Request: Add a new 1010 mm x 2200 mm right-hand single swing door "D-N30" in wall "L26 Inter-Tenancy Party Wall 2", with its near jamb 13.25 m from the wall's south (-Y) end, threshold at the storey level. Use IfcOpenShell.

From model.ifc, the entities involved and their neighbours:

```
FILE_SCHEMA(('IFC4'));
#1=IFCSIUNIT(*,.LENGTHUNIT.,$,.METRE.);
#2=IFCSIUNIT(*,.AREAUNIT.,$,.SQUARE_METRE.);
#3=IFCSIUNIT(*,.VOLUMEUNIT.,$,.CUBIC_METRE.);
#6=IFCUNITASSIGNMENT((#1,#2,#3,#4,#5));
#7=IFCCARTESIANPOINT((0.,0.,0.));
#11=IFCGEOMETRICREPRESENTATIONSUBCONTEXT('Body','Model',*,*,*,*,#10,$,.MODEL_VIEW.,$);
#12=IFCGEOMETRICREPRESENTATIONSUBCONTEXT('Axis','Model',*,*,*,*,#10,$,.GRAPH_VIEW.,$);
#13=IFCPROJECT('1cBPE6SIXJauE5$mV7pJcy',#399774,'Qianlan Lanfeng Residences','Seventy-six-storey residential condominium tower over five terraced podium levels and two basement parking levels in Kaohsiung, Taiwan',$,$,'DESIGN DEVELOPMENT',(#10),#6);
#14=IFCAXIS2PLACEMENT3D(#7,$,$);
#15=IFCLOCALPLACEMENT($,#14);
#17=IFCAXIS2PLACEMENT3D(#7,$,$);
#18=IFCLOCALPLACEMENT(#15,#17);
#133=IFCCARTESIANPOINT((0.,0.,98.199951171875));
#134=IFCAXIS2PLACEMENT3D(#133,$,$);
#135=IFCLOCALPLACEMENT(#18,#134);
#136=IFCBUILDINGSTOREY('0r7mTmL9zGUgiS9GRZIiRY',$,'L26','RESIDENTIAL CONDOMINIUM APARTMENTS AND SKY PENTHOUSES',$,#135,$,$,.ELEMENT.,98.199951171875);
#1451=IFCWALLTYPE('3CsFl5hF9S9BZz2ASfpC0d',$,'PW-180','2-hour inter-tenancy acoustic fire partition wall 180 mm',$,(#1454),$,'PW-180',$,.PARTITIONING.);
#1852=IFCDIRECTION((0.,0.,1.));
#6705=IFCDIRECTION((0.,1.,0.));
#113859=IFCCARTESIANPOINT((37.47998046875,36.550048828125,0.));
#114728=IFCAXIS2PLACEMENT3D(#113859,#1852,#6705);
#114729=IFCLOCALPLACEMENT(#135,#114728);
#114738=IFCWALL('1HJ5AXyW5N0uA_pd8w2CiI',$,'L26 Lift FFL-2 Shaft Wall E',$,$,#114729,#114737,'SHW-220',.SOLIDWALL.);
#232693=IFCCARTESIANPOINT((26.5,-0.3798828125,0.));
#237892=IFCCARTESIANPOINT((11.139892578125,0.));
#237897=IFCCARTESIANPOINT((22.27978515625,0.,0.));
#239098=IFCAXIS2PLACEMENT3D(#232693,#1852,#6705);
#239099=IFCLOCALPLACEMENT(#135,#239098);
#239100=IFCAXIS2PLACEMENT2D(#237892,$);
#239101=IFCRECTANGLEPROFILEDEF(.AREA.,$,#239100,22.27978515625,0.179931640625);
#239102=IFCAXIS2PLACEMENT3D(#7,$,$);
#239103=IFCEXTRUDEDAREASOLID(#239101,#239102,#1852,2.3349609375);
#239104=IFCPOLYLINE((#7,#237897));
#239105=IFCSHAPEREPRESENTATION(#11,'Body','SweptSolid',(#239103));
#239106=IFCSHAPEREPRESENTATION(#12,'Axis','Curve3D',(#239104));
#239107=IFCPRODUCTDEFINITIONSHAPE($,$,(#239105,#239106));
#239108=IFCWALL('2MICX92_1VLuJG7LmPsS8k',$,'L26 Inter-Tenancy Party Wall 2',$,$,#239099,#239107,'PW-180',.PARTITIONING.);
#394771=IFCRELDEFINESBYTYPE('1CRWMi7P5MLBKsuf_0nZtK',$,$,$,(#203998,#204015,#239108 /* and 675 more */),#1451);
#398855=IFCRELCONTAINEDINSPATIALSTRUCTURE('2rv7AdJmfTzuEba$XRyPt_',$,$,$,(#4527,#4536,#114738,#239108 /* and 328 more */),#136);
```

```python
import numpy as np
import ifcopenshell
import ifcopenshell.api.feature
import ifcopenshell.api.geometry
import ifcopenshell.api.root
import ifcopenshell.api.spatial
import ifcopenshell.geom
import ifcopenshell.util.element
import ifcopenshell.util.placement
import ifcopenshell.util.representation
import ifcopenshell.util.shape
import ifcopenshell.util.unit

model = ifcopenshell.open("model.ifc")
unit_scale = ifcopenshell.util.unit.calculate_unit_scale(model)
settings = ifcopenshell.geom.settings()


def volume(element):
    """Net volume in cubic metres, openings subtracted."""
    shape = ifcopenshell.geom.create_shape(settings, element)
    return ifcopenshell.util.shape.get_volume(shape.geometry)


wall = model.by_id(239108)
storey = ifcopenshell.util.element.get_container(wall, ifc_class="IfcBuildingStorey")
context = ifcopenshell.util.representation.get_context(model, "Model", "Body", "MODEL_VIEW")
before = volume(wall)

width, height, from_end, sill = 1.01, 2.2, 13.25, 0.0  # metres

# The wall runs along its own X axis, and the end named is its -X end.
wall_shape = ifcopenshell.geom.create_shape(settings, wall)
x, y, z = ifcopenshell.util.shape.get_vertices(wall_shape.geometry).T
start = x.min() + from_end
face, thickness = float(y.min()), float(y.max() - y.min())
wall_matrix = ifcopenshell.util.placement.get_local_placement(wall.ObjectPlacement)
level = ifcopenshell.util.placement.get_local_placement(storey.ObjectPlacement)[2, 3]


def in_wall(x, y):
    """Placement at x, y metres in the wall's axes, at sill height."""
    matrix = wall_matrix.copy()
    matrix[:, 3] = wall_matrix @ np.array([x / unit_scale, y / unit_scale, 0.0, 1.0])
    matrix[2, 3] = level + sill / unit_scale
    return matrix


# Opening: a box that overshoots both wall faces by 50 mm.
opening = ifcopenshell.api.root.create_entity(model, ifc_class="IfcOpeningElement", predefined_type="OPENING")
box = ifcopenshell.api.geometry.add_wall_representation(
    model, context=context, length=width, height=height, thickness=thickness + 0.1
)
ifcopenshell.api.geometry.assign_representation(model, product=opening, representation=box)
ifcopenshell.api.geometry.edit_object_placement(model, product=opening, matrix=in_wall(start, face - 0.05), is_si=False)
ifcopenshell.api.feature.add_feature(model, feature=opening, element=wall)

door = ifcopenshell.api.root.create_entity(model, ifc_class="IfcDoor", name="D-N30", predefined_type="DOOR")
door.OverallWidth, door.OverallHeight = width / unit_scale, height / unit_scale
door.OperationType = "SINGLE_SWING_RIGHT"
body = ifcopenshell.api.geometry.add_door_representation(
    model,
    context=context,
    overall_width=door.OverallWidth,
    overall_height=door.OverallHeight,
    operation_type="SINGLE_SWING_RIGHT",
    lining_properties={"LiningDepth": thickness / unit_scale, "ThresholdDepth": thickness / unit_scale},
)
ifcopenshell.api.geometry.assign_representation(model, product=door, representation=body)
ifcopenshell.api.spatial.assign_container(model, products=[door], relating_structure=storey)
ifcopenshell.api.feature.add_filling(model, opening=opening, element=door)

# The lining spans the wall, so the door starts at the wall face.
ifcopenshell.api.geometry.edit_object_placement(model, product=door, matrix=in_wall(start, face), is_si=False)

after = volume(wall)

print(f"wall volume {before:.3f} -> {after:.3f} m3")

model.write("model_v2.ifc")
```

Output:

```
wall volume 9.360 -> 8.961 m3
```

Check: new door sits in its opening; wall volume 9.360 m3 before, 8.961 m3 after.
